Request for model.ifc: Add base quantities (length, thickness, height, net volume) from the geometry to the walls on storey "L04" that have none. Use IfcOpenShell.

First a look at what the model holds.

```python
import ifcopenshell
import ifcopenshell.util.element
import ifcopenshell.util.unit

model = ifcopenshell.open("model.ifc")
print(model.schema)
for unit_type in ("LENGTHUNIT", "AREAUNIT", "VOLUMEUNIT"):
    print(unit_type, ifcopenshell.util.unit.calculate_unit_scale(model, unit_type))
storey = next(s for s in model.by_type("IfcBuildingStorey") if s.Name == "L04")
walls = [e for e in ifcopenshell.util.element.get_decomposition(storey) if e.is_a("IfcWall")]
for e in sorted(walls, key=lambda e: e.id()):
    print(e.id(), e.is_a(), e.Name, list(ifcopenshell.util.element.get_psets(e, qtos_only=True)), sep=" | ")
```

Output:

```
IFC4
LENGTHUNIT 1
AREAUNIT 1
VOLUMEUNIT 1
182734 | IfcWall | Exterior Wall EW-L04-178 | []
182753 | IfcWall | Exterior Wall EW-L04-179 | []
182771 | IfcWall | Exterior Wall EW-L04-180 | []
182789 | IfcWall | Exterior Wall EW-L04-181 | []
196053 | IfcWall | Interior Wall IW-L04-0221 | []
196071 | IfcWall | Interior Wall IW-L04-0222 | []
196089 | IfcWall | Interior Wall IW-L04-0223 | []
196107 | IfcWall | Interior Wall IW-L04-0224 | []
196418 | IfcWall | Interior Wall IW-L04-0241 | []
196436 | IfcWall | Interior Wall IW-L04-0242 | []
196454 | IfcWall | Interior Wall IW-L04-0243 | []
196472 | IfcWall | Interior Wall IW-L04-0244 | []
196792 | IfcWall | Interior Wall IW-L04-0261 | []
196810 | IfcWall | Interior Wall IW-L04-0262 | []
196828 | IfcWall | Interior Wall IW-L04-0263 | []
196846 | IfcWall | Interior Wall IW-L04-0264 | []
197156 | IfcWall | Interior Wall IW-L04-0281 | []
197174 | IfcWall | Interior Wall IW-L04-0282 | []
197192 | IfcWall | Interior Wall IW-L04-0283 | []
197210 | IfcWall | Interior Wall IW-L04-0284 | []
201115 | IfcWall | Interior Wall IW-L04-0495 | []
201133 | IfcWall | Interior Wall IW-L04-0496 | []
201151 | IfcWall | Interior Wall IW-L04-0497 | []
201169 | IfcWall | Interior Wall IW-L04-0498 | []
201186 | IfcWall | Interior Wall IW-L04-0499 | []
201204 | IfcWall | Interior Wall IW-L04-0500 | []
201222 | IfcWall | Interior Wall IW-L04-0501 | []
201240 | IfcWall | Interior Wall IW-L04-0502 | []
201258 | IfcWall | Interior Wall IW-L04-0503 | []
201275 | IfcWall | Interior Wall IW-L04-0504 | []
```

```python
import ifcopenshell
import ifcopenshell.api.pset
import ifcopenshell.geom
import ifcopenshell.util.element
import ifcopenshell.util.shape
import ifcopenshell.util.unit

model = ifcopenshell.open("model.ifc")
unit_scale = ifcopenshell.util.unit.calculate_unit_scale(model)
volume_scale = ifcopenshell.util.unit.calculate_unit_scale(model, "VOLUMEUNIT")
settings = ifcopenshell.geom.settings()

storey = next(s for s in model.by_type("IfcBuildingStorey") if s.Name == "L04")
walls = [e for e in ifcopenshell.util.element.get_decomposition(storey) if e.is_a("IfcWall")]

for e in sorted(walls, key=lambda e: e.id()):
    if ifcopenshell.util.element.get_psets(e, qtos_only=True, should_inherit=False):
        continue
    # Geometry comes back in metres, in the element's own axes.
    shape = ifcopenshell.geom.create_shape(settings, e)
    values = {
        "Length": ifcopenshell.util.shape.get_x(shape.geometry) / unit_scale,
        "Width": ifcopenshell.util.shape.get_y(shape.geometry) / unit_scale,
        "Height": ifcopenshell.util.shape.get_z(shape.geometry) / unit_scale,
        "NetVolume": ifcopenshell.util.shape.get_volume(shape.geometry) / volume_scale,
    }
    qto = ifcopenshell.api.pset.add_qto(model, product=e, name="Qto_WallBaseQuantities")
    ifcopenshell.api.pset.edit_qto(model, qto=qto, properties=values)
    print(e.id(), {k: round(v, 3) for k, v in values.items()})

model.write("model_rev.ifc")
```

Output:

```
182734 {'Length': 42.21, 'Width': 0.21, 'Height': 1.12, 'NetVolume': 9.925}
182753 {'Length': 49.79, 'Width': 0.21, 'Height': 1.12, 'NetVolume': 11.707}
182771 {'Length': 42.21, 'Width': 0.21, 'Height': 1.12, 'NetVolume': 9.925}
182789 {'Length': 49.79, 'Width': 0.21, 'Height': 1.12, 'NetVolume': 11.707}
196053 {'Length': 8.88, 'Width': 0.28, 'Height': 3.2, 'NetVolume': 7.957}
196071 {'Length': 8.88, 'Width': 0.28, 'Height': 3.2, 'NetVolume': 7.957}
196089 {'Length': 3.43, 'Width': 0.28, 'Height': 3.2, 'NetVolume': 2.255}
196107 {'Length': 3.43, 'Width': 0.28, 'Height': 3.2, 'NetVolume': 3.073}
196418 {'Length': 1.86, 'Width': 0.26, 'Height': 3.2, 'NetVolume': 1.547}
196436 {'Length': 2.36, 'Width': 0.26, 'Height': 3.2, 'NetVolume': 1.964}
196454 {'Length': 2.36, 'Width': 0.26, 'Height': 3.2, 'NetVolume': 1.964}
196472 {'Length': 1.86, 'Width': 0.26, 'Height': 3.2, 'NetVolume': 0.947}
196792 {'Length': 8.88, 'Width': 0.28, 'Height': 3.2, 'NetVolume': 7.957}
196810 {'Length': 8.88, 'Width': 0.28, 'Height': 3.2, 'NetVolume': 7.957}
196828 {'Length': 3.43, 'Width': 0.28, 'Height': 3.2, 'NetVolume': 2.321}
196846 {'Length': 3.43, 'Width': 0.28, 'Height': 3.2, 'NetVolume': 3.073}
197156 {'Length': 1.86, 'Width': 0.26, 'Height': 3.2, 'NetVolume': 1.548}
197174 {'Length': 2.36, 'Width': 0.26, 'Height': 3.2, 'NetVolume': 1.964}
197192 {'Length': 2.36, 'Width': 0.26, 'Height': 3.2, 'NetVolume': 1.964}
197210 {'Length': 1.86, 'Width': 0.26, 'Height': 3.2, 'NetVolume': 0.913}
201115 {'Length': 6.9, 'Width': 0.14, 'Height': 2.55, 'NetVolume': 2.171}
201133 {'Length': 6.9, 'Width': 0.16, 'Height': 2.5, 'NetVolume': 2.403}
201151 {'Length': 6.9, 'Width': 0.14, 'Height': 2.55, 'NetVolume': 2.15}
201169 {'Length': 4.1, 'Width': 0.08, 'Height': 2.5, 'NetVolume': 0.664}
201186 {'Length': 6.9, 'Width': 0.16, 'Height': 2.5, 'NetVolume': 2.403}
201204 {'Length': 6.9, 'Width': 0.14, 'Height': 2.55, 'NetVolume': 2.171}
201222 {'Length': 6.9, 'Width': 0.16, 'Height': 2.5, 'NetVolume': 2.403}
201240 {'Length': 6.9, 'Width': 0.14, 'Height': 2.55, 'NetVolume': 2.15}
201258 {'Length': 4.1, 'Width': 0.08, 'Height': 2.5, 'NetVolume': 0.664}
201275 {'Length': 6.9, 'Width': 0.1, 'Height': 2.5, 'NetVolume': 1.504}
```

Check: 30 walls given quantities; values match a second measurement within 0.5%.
